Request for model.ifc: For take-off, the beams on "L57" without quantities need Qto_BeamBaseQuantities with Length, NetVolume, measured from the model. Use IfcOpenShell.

First a look at what the model holds.

```python
import ifcopenshell
import ifcopenshell.util.element
import ifcopenshell.util.unit

model = ifcopenshell.open("model.ifc")
print(model.schema)
for unit_type in ("LENGTHUNIT", "AREAUNIT", "VOLUMEUNIT"):
    print(unit_type, ifcopenshell.util.unit.calculate_unit_scale(model, unit_type))
storey = next(s for s in model.by_type("IfcBuildingStorey") if s.Name == "L57")
beams = [e for e in ifcopenshell.util.element.get_decomposition(storey) if e.is_a("IfcBeam")]
for e in sorted(beams, key=lambda e: e.id()):
    print(e.id(), e.is_a(), e.Name, list(ifcopenshell.util.element.get_psets(e, qtos_only=True)), sep=" | ")
```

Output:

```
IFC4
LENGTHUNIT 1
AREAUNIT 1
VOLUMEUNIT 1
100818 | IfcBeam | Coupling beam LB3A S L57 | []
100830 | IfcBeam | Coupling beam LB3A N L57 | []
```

```python
import ifcopenshell
import ifcopenshell.api.pset
import ifcopenshell.geom
import ifcopenshell.util.element
import ifcopenshell.util.shape
import ifcopenshell.util.unit

model = ifcopenshell.open("model.ifc")
unit_scale = ifcopenshell.util.unit.calculate_unit_scale(model)
volume_scale = ifcopenshell.util.unit.calculate_unit_scale(model, "VOLUMEUNIT")
settings = ifcopenshell.geom.settings()

storey = next(s for s in model.by_type("IfcBuildingStorey") if s.Name == "L57")
beams = [e for e in ifcopenshell.util.element.get_decomposition(storey) if e.is_a("IfcBeam")]

for e in sorted(beams, key=lambda e: e.id()):
    if ifcopenshell.util.element.get_psets(e, qtos_only=True, should_inherit=False):
        continue
    # Geometry comes back in metres, in the element's own axes.
    shape = ifcopenshell.geom.create_shape(settings, e)
    values = {
        "Length": ifcopenshell.util.shape.get_max_xyz(shape.geometry) / unit_scale,
        "NetVolume": ifcopenshell.util.shape.get_volume(shape.geometry) / volume_scale,
    }
    qto = ifcopenshell.api.pset.add_qto(model, product=e, name="Qto_BeamBaseQuantities")
    ifcopenshell.api.pset.edit_qto(model, qto=qto, properties=values)
    print(e.id(), {k: round(v, 3) for k, v in values.items()})

model.write("model_rev.ifc")
```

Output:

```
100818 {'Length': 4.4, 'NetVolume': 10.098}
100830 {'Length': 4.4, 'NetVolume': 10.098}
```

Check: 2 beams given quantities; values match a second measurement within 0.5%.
